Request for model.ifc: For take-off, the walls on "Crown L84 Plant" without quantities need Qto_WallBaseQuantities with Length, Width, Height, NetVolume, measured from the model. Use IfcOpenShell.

First a look at what the model holds.

```python
import ifcopenshell
import ifcopenshell.util.element
import ifcopenshell.util.unit

model = ifcopenshell.open("model.ifc")
print(model.schema)
for unit_type in ("LENGTHUNIT", "AREAUNIT", "VOLUMEUNIT"):
    print(unit_type, ifcopenshell.util.unit.calculate_unit_scale(model, unit_type))
storey = next(s for s in model.by_type("IfcBuildingStorey") if s.Name == "Crown L84 Plant")
walls = [e for e in ifcopenshell.util.element.get_decomposition(storey) if e.is_a("IfcWall")]
for e in sorted(walls, key=lambda e: e.id()):
    print(e.id(), e.is_a(), e.Name, list(ifcopenshell.util.element.get_psets(e, qtos_only=True)), sep=" | ")
```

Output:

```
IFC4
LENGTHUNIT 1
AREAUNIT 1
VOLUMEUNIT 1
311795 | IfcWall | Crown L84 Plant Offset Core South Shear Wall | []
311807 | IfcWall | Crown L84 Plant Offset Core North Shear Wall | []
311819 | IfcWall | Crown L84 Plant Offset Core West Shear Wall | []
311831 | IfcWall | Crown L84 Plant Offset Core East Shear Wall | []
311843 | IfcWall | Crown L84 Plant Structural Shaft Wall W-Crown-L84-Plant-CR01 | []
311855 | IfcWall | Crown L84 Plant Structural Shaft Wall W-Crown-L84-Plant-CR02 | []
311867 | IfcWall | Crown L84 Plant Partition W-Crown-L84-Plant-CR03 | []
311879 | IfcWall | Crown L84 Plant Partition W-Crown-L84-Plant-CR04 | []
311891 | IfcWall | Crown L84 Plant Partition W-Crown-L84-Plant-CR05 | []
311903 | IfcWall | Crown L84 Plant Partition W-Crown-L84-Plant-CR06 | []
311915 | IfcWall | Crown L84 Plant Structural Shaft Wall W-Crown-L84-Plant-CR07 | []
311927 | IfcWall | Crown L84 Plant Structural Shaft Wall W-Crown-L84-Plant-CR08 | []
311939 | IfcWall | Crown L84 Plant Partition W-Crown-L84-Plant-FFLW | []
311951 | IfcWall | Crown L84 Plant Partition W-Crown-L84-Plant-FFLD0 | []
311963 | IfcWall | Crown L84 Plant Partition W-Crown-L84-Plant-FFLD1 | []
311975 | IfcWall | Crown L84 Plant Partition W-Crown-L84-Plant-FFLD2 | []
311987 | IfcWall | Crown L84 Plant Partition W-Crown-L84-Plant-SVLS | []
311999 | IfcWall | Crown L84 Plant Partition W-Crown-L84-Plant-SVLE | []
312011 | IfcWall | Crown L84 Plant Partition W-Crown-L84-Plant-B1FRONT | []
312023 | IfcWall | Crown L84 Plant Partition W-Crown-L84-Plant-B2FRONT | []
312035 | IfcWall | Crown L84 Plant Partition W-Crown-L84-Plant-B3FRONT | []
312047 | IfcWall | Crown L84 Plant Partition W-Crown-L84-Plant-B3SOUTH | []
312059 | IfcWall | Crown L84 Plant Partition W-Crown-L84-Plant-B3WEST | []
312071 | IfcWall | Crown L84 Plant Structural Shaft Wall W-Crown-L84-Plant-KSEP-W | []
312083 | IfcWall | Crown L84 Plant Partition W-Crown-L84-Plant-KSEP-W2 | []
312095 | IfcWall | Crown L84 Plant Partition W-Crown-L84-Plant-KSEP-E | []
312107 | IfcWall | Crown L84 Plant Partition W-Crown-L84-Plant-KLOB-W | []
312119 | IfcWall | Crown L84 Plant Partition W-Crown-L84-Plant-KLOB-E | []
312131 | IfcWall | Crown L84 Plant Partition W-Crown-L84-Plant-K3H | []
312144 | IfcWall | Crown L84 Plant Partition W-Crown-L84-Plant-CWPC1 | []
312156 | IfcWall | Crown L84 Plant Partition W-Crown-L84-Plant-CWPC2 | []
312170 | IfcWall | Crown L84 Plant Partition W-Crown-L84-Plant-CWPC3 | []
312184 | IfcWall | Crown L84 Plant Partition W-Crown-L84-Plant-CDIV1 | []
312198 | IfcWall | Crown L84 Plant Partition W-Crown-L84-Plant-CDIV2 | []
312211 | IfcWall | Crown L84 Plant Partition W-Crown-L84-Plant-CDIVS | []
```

```python
import ifcopenshell
import ifcopenshell.api.pset
import ifcopenshell.geom
import ifcopenshell.util.element
import ifcopenshell.util.shape
import ifcopenshell.util.unit

model = ifcopenshell.open("model.ifc")
unit_scale = ifcopenshell.util.unit.calculate_unit_scale(model)
volume_scale = ifcopenshell.util.unit.calculate_unit_scale(model, "VOLUMEUNIT")
settings = ifcopenshell.geom.settings()

storey = next(s for s in model.by_type("IfcBuildingStorey") if s.Name == "Crown L84 Plant")
walls = [e for e in ifcopenshell.util.element.get_decomposition(storey) if e.is_a("IfcWall")]

for e in sorted(walls, key=lambda e: e.id()):
    if ifcopenshell.util.element.get_psets(e, qtos_only=True, should_inherit=False):
        continue
    # Geometry comes back in metres, in the element's own axes.
    shape = ifcopenshell.geom.create_shape(settings, e)
    values = {
        "Length": ifcopenshell.util.shape.get_x(shape.geometry) / unit_scale,
        "Width": ifcopenshell.util.shape.get_y(shape.geometry) / unit_scale,
        "Height": ifcopenshell.util.shape.get_z(shape.geometry) / unit_scale,
        "NetVolume": ifcopenshell.util.shape.get_volume(shape.geometry) / volume_scale,
    }
    qto = ifcopenshell.api.pset.add_qto(model, product=e, name="Qto_WallBaseQuantities")
    ifcopenshell.api.pset.edit_qto(model, qto=qto, properties=values)
    print(e.id(), {k: round(v, 3) for k, v in values.items()})

model.write("model-out.ifc")
```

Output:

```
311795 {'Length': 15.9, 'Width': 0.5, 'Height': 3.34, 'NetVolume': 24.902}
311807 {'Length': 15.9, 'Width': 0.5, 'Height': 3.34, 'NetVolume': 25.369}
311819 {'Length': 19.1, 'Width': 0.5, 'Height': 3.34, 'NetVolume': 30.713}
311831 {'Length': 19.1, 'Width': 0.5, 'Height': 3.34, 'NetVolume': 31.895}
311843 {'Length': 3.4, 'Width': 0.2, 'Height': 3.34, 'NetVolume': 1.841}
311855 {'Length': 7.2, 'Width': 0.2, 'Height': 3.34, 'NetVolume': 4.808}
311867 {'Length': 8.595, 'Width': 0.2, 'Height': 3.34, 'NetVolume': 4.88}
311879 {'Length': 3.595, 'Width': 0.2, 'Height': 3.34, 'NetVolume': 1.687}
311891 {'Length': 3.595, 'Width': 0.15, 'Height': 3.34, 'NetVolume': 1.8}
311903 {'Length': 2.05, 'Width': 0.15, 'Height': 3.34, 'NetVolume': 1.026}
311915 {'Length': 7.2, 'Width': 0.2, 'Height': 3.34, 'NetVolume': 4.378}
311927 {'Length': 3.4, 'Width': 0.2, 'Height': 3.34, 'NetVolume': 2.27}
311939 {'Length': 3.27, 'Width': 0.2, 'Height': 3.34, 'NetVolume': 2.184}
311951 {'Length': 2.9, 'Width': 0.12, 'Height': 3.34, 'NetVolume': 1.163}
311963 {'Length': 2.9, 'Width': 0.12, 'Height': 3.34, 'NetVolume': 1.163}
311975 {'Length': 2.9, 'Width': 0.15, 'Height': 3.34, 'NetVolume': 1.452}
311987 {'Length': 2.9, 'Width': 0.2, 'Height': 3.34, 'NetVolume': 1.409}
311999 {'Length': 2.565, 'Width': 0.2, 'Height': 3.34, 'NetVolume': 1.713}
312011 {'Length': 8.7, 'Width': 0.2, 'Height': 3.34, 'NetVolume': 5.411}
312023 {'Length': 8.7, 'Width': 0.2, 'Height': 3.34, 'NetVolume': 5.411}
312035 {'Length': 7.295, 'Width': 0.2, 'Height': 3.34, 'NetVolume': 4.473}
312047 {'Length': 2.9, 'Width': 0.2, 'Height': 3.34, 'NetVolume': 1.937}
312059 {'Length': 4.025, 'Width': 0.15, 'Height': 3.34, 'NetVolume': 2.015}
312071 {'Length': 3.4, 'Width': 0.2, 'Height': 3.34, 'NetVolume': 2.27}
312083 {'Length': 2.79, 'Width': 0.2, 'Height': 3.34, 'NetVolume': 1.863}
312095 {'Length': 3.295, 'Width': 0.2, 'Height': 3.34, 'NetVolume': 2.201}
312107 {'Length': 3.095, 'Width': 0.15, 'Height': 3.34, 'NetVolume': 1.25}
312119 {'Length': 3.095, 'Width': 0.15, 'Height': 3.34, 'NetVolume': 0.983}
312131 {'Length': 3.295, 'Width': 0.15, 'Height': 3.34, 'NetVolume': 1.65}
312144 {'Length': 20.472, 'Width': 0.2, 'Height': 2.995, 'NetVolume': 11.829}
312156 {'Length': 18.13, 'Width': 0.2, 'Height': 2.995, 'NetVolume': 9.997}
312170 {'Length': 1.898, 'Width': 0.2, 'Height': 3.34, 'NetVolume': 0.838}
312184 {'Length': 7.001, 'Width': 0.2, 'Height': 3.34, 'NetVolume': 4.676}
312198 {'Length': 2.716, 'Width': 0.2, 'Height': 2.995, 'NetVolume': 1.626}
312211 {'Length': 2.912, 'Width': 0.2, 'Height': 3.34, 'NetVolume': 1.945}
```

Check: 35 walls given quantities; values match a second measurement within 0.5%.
